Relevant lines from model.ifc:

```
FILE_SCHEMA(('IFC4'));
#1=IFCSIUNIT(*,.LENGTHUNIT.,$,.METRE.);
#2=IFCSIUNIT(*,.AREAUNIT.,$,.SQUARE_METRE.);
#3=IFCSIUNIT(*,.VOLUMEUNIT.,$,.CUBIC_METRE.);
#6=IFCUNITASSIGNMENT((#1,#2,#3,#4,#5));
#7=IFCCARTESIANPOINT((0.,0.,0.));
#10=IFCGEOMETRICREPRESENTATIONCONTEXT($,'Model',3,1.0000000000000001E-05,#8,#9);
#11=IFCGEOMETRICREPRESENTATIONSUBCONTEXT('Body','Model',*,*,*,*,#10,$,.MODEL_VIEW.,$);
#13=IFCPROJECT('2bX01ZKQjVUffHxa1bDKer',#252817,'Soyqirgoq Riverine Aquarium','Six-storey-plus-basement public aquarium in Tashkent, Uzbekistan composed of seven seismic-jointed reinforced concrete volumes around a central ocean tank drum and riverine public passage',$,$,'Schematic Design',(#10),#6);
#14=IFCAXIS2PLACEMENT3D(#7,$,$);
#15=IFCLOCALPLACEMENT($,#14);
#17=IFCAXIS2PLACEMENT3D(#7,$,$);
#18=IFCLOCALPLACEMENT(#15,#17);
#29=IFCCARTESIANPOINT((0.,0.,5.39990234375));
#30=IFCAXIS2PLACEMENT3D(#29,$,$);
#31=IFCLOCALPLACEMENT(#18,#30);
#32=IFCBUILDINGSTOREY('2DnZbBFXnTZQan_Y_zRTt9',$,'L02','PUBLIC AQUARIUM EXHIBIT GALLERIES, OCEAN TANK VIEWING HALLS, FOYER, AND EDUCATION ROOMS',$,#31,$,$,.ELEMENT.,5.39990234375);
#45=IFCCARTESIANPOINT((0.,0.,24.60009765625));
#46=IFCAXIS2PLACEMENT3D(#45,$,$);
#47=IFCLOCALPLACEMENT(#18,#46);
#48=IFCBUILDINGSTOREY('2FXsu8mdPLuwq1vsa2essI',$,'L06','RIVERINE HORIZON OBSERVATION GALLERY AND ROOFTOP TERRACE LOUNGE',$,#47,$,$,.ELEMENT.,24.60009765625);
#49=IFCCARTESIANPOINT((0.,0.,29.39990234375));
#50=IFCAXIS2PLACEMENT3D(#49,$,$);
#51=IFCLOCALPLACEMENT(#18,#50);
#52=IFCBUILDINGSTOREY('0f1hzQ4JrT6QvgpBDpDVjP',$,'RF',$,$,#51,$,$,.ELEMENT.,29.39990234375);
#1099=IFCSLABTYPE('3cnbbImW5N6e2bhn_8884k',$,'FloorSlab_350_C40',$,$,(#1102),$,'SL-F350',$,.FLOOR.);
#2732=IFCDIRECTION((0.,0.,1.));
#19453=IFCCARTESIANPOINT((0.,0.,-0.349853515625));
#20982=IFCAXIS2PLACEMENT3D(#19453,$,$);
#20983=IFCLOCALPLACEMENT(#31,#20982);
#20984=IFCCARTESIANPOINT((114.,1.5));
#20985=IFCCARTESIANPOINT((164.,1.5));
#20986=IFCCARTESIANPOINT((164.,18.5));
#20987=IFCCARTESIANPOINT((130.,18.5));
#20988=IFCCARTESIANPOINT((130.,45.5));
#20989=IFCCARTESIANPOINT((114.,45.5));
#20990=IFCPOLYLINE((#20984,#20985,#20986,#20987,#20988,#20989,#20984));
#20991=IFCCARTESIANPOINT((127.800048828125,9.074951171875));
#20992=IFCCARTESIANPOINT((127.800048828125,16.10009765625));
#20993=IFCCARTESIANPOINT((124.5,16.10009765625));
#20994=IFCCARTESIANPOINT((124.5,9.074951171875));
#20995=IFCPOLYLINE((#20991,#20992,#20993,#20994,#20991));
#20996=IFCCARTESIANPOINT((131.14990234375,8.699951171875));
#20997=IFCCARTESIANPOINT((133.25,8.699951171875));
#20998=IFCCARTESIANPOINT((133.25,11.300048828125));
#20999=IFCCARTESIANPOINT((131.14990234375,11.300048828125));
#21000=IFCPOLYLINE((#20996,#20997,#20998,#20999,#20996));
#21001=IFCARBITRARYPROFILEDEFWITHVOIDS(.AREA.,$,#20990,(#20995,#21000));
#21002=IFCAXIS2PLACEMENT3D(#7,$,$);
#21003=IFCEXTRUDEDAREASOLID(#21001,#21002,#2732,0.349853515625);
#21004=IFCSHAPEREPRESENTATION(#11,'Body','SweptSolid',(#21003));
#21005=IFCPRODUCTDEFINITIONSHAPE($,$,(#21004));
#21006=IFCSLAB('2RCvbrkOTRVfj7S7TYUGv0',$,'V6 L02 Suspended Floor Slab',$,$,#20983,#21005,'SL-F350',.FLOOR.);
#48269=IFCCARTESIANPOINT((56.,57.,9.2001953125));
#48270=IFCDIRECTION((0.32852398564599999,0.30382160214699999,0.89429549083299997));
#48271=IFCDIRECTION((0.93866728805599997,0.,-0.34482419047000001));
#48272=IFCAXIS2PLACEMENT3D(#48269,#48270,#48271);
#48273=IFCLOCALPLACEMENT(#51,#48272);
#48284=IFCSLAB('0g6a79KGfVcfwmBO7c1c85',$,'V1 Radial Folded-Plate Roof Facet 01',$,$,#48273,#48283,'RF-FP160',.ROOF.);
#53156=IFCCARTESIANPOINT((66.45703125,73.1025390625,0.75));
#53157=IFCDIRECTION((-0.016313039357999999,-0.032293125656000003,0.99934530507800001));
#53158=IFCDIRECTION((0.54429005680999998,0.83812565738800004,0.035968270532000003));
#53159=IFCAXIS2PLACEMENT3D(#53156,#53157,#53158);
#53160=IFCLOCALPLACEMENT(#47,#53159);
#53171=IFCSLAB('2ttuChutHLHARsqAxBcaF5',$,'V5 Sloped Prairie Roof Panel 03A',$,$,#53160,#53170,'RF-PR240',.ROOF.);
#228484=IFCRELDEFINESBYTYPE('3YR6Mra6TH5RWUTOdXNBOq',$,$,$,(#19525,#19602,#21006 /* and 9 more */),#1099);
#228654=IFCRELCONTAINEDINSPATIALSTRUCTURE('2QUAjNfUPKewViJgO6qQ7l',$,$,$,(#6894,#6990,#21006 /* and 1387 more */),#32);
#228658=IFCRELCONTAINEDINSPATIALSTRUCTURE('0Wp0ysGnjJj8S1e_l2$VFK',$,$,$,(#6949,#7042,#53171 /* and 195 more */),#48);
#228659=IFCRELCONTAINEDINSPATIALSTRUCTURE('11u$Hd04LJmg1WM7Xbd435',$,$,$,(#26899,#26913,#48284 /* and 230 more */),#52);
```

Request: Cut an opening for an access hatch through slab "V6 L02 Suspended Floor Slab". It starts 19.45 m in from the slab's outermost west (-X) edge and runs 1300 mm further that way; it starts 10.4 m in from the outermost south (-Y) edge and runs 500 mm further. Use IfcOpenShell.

```python
import numpy as np
import ifcopenshell
import ifcopenshell.api.feature
import ifcopenshell.api.geometry
import ifcopenshell.api.root
import ifcopenshell.geom
import ifcopenshell.util.placement
import ifcopenshell.util.representation
import ifcopenshell.util.shape
import ifcopenshell.util.unit

model = ifcopenshell.open("model.ifc")
unit_scale = ifcopenshell.util.unit.calculate_unit_scale(model)
settings = ifcopenshell.geom.settings()


def volume(element):
    """Net volume in cubic metres, openings subtracted."""
    shape = ifcopenshell.geom.create_shape(settings, element)
    return ifcopenshell.util.shape.get_volume(shape.geometry)


slab = model.by_guid("2RCvbrkOTRVfj7S7TYUGv0")
before = volume(slab)

# Extent in the slab's own axes, in metres. The edges named are its -X and -Y sides.
slab_shape = ifcopenshell.geom.create_shape(settings, slab)
vertices = ifcopenshell.util.shape.get_vertices(slab_shape.geometry)
x_min, y_min, bottom = vertices.min(axis=0)
top = vertices[:, 2].max()

opening = ifcopenshell.api.root.create_entity(model, ifc_class="IfcOpeningElement", name="Access hatch opening", predefined_type="OPENING")
context = ifcopenshell.util.representation.get_context(model, "Model", "Body", "MODEL_VIEW")
width, depth = 1.3, 0.5
outline = [(0.0, 0.0), (width, 0.0), (width, depth), (0.0, depth), (0.0, 0.0)]
# Overshoot both faces by 50 mm so the cut is clean.
shape = ifcopenshell.api.geometry.add_slab_representation(
    model, context=context, depth=top - bottom + 0.1, polyline=outline
)
ifcopenshell.api.geometry.assign_representation(model, product=opening, representation=shape)

matrix = ifcopenshell.util.placement.get_local_placement(slab.ObjectPlacement)
matrix[:, 3] = matrix @ np.append(np.array([x_min + 19.45, y_min + 10.4, bottom - 0.05]) / unit_scale, 1.0)
ifcopenshell.api.geometry.edit_object_placement(model, product=opening, matrix=matrix, is_si=False)
ifcopenshell.api.feature.add_feature(model, feature=opening, element=slab)

after = volume(slab)

print(f"slab volume {before:.3f} -> {after:.3f} m3")

model.write("model_edited.ifc")
```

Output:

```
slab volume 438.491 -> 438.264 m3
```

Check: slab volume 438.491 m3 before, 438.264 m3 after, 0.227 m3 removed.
